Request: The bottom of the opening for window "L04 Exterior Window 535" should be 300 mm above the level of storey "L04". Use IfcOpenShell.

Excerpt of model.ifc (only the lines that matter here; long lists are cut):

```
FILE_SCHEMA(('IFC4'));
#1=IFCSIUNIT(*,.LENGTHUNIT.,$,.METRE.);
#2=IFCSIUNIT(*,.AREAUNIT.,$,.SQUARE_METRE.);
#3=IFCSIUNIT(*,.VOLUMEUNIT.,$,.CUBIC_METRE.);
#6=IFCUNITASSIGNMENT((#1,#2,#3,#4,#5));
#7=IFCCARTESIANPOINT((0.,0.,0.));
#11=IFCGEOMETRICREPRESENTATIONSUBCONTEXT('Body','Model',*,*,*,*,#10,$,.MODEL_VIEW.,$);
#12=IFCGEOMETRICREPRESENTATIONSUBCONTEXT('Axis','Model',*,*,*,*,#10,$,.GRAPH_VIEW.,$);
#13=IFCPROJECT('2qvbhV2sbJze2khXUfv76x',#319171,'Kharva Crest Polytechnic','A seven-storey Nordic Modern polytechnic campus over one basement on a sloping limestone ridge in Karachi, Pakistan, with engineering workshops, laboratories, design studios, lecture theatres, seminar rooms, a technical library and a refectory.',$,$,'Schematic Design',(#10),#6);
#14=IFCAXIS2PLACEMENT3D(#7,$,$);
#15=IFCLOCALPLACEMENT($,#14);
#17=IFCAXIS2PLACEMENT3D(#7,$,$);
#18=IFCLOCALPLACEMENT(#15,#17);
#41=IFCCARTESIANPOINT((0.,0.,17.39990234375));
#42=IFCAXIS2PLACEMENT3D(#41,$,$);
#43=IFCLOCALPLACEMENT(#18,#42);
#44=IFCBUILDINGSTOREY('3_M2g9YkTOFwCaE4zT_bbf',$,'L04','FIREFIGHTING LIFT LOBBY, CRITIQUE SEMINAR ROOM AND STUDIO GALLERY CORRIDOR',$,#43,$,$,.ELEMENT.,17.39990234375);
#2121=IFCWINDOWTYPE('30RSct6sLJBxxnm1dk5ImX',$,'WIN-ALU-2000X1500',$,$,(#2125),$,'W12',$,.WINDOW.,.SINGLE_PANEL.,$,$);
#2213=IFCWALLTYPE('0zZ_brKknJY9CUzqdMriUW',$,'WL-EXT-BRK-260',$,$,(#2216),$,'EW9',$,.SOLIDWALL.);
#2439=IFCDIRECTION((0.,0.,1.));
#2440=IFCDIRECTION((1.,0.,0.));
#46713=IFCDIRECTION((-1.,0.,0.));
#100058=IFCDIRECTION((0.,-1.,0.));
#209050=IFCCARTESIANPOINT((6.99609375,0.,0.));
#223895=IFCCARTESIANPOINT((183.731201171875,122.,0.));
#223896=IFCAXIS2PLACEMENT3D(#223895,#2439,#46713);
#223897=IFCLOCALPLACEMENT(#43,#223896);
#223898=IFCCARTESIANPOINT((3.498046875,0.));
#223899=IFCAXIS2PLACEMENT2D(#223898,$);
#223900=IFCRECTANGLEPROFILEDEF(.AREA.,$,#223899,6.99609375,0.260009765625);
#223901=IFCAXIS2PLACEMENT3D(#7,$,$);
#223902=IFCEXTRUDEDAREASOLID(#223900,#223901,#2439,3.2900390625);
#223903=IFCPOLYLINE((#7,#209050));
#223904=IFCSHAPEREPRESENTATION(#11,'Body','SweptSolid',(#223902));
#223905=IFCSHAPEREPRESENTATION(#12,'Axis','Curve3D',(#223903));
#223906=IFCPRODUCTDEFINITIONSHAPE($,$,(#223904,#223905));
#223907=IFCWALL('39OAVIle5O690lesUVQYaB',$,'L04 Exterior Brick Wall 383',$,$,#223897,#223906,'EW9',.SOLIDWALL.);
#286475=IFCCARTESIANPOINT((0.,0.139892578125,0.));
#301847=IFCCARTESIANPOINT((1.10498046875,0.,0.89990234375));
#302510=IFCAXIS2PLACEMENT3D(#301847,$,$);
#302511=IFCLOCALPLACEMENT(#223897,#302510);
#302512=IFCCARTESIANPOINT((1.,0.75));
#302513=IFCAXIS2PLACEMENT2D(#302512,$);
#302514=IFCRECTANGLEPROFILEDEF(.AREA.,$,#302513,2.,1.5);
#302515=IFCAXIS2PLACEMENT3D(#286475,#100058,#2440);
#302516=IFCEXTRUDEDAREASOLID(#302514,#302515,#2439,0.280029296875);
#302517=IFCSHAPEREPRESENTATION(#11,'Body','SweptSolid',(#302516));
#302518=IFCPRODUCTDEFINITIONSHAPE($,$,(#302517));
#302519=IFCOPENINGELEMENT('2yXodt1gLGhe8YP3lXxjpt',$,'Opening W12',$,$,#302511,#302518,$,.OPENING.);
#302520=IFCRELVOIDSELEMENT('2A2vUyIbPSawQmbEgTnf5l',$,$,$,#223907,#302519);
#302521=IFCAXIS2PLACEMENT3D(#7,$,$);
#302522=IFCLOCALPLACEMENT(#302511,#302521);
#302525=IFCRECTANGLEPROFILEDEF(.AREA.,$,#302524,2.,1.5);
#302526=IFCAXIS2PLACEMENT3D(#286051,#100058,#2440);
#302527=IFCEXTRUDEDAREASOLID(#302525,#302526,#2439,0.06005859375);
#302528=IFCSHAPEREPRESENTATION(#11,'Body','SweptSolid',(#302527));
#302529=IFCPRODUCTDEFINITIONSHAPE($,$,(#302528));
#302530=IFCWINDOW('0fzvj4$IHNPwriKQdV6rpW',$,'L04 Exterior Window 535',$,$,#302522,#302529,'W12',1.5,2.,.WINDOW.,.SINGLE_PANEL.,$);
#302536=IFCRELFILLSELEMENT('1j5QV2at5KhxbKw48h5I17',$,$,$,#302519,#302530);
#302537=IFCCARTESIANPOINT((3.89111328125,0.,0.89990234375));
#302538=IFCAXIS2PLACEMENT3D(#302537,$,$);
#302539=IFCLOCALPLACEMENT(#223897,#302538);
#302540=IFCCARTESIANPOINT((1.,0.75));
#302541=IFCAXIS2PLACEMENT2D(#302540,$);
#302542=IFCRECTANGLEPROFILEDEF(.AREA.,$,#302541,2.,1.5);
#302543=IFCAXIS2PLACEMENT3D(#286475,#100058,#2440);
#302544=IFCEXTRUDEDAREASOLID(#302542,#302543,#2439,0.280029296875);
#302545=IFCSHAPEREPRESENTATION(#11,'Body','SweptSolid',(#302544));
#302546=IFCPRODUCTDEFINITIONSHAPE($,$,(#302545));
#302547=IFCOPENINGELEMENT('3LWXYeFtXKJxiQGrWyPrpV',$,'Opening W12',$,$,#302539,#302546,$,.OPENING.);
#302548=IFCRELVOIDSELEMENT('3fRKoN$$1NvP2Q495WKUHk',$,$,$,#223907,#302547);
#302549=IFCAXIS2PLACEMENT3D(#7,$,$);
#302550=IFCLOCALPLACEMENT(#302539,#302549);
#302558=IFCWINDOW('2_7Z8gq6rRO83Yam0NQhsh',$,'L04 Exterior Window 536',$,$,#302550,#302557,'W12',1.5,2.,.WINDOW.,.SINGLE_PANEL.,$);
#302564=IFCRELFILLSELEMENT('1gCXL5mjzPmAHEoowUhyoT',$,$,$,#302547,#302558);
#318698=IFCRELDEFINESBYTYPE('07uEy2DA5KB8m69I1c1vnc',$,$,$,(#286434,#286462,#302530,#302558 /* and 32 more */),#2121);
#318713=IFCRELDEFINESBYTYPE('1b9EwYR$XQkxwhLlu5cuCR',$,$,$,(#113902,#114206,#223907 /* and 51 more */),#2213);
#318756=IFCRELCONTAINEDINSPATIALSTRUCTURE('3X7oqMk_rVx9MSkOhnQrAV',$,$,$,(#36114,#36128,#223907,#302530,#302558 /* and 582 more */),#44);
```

```python
import numpy as np
import ifcopenshell
import ifcopenshell.api.geometry
import ifcopenshell.geom
import ifcopenshell.util.element
import ifcopenshell.util.placement
import ifcopenshell.util.shape
import ifcopenshell.util.unit

model = ifcopenshell.open("model.ifc")
unit_scale = ifcopenshell.util.unit.calculate_unit_scale(model)

window = model.by_guid("0fzvj4$IHNPwriKQdV6rpW")
opening = window.FillsVoids[0].RelatingOpeningElement
storey = ifcopenshell.util.element.get_container(window, ifc_class="IfcBuildingStorey")
level = ifcopenshell.util.placement.get_local_placement(storey.ObjectPlacement)[2, 3]

# The opening's origin need not be at the sill, so measure its lowest point.
shape = ifcopenshell.geom.create_shape(ifcopenshell.geom.settings(), opening)
bottom = ifcopenshell.util.shape.get_shape_bottom_elevation(shape, shape.geometry) / unit_scale
dz = level + 0.3 - bottom

shift = np.array([0.0, 0.0, dz])
# The window is placed relative to its opening, so it follows when the opening moves.
matrix = ifcopenshell.util.placement.get_local_placement(opening.ObjectPlacement)
matrix[:3, 3] += shift
ifcopenshell.api.geometry.edit_object_placement(
    model, product=opening, matrix=matrix, is_si=False, should_transform_children=True
)

print(f"moved by {dz * unit_scale:+.3f} m")

model.write("model_updated.ifc")
```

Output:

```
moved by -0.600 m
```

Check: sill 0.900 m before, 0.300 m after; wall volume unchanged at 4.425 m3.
